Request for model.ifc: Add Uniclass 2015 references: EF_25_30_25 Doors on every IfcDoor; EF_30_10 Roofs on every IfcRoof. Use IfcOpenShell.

First a look at what the model holds.

```python
import ifcopenshell

model = ifcopenshell.open("model.ifc")
print(model.schema)
print("classifications:", [c.Name for c in model.by_type("IfcClassification")])
for ifc_class in ("IfcDoor", "IfcRoof", "IfcStair", "IfcWall", "IfcWindow"):
    print(ifc_class, len(model.by_type(ifc_class)))
```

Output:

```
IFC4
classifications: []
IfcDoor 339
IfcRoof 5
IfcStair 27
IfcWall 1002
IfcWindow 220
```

```python
import ifcopenshell
import ifcopenshell.api.classification

model = ifcopenshell.open("model.ifc")

system = ifcopenshell.api.classification.add_classification(model, classification="Uniclass 2015")

codes = {
    "IfcDoor": ("EF_25_30_25", "Doors"),
    "IfcRoof": ("EF_30_10", "Roofs"),
}
for ifc_class, (code, name) in codes.items():
    products = model.by_type(ifc_class)
    ifcopenshell.api.classification.add_reference(
        model, products=products, classification=system, identification=code, name=name
    )
    print(code, len(products))

model.write("model_edited.ifc")
```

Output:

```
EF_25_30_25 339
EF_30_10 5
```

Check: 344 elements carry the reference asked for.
